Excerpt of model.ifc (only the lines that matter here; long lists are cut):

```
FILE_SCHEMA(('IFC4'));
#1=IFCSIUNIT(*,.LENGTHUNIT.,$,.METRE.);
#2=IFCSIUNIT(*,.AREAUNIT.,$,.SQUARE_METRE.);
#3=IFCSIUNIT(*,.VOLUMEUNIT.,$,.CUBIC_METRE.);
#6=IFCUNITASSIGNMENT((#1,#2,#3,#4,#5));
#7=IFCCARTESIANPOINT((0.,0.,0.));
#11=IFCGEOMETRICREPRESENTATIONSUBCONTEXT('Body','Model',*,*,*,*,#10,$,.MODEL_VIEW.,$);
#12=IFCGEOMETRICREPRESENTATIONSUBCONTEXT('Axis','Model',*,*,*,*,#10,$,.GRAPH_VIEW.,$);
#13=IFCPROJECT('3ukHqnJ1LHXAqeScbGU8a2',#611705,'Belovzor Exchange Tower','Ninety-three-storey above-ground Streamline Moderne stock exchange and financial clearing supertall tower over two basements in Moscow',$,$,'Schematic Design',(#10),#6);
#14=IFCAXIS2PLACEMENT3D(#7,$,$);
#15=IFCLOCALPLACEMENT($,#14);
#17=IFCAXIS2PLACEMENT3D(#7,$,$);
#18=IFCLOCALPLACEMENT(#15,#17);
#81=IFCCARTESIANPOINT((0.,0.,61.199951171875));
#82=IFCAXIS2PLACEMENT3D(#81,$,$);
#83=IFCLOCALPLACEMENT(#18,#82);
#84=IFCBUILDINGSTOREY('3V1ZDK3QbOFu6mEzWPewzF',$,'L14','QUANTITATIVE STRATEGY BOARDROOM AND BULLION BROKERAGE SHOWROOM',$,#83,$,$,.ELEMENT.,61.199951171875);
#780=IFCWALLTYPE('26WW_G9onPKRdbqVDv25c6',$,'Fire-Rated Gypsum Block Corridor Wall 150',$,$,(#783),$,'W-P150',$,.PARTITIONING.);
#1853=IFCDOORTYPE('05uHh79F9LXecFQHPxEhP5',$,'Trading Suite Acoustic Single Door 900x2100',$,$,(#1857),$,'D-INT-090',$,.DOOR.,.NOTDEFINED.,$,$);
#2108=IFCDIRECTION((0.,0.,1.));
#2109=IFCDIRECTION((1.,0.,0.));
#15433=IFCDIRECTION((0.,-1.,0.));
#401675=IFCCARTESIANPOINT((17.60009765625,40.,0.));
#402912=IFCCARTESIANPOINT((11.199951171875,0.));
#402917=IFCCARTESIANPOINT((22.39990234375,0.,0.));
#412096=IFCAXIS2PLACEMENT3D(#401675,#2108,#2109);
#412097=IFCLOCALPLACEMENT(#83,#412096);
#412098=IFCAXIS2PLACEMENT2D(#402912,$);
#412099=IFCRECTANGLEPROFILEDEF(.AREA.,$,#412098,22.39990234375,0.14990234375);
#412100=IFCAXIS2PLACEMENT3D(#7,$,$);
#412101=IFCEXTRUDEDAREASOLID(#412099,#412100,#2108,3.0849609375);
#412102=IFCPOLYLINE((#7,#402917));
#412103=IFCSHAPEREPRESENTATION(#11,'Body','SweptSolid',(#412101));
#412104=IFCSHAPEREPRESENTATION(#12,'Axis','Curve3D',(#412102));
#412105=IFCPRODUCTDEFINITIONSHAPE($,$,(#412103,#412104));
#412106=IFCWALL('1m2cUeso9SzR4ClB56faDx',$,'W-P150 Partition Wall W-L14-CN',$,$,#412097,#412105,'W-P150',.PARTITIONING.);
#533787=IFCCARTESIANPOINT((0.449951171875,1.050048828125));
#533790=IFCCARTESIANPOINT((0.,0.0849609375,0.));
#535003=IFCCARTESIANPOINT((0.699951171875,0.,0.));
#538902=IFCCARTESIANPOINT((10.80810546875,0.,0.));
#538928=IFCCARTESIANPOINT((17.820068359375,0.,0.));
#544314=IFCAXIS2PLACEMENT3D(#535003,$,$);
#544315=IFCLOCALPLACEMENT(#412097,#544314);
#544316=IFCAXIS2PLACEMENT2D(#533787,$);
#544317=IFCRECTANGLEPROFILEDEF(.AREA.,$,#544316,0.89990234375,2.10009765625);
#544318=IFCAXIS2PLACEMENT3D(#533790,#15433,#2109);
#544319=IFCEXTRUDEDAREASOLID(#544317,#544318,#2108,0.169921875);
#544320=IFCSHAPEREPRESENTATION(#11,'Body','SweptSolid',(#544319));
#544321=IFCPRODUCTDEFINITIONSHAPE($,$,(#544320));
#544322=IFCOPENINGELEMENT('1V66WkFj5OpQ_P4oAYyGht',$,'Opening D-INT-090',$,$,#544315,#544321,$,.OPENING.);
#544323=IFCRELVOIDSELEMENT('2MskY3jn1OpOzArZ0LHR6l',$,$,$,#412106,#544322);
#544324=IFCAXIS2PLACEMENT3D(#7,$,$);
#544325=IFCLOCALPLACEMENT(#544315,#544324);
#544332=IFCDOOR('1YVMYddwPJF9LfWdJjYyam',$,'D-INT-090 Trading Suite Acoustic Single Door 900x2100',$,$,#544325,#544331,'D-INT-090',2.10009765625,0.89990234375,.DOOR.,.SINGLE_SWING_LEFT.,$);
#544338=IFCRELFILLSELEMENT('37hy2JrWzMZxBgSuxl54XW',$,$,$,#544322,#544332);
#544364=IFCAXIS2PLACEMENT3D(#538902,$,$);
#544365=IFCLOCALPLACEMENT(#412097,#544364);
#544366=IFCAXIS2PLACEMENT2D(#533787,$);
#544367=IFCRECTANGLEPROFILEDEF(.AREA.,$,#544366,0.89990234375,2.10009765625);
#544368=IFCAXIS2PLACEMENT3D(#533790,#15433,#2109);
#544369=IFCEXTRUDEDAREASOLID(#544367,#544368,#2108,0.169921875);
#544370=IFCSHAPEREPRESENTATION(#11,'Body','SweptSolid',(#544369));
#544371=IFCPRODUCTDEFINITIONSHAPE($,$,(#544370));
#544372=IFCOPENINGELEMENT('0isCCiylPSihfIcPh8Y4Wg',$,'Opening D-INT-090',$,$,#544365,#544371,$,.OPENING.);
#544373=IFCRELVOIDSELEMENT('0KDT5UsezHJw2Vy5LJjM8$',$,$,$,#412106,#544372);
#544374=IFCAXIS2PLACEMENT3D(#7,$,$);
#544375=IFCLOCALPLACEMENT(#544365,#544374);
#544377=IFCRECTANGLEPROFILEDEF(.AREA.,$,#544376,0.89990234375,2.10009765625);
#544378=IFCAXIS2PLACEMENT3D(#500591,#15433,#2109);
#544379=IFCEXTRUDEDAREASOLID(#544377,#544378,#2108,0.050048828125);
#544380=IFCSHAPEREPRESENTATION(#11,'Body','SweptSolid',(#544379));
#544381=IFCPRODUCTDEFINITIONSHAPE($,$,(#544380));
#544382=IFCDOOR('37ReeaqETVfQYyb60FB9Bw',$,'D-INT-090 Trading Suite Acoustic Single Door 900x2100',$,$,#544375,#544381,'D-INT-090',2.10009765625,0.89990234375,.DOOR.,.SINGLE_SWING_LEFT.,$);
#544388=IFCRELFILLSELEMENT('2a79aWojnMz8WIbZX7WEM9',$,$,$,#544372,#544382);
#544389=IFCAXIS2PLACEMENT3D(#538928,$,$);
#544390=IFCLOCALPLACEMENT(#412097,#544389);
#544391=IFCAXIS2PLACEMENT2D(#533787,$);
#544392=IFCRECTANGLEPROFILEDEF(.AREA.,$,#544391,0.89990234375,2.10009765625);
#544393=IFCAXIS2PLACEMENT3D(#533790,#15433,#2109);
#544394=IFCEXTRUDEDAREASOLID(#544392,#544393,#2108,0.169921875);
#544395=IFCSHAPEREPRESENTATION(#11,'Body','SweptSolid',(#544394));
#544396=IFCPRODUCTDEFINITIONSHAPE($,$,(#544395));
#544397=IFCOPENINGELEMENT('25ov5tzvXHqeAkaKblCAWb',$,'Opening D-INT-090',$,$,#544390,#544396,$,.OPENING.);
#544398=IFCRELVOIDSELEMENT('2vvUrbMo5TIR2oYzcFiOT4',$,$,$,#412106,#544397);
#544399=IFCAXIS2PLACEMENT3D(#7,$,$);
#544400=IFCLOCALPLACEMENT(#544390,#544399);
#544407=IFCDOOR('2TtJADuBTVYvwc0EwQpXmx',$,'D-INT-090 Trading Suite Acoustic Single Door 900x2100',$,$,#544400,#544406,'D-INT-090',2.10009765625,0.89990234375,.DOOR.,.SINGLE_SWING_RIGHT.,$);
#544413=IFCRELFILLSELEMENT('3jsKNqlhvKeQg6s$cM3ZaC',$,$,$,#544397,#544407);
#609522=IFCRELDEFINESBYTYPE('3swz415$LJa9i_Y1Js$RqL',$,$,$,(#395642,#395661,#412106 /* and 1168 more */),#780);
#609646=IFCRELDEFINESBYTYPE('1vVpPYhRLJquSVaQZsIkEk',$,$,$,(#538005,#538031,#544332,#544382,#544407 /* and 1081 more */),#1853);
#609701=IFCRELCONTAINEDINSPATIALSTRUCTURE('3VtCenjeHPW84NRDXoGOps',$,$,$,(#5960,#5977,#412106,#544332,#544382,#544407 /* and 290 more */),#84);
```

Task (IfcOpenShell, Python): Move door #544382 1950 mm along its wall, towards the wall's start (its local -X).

```python
import ifcopenshell
import ifcopenshell.api.geometry
import ifcopenshell.util.placement
import ifcopenshell.util.unit

model = ifcopenshell.open("model.ifc")
unit_scale = ifcopenshell.util.unit.calculate_unit_scale(model)

door = model.by_guid("37ReeaqETVfQYyb60FB9Bw")
opening = door.FillsVoids[0].RelatingOpeningElement
wall = opening.VoidsElements[0].RelatingBuildingElement

wall_matrix = ifcopenshell.util.placement.get_local_placement(wall.ObjectPlacement)
shift = wall_matrix[:3, 0] * -1.95 / unit_scale
before = ifcopenshell.util.placement.get_local_placement(door.ObjectPlacement)[:3, 3].copy()

# The door is placed relative to its opening, so it follows when the opening moves.
matrix = ifcopenshell.util.placement.get_local_placement(opening.ObjectPlacement)
matrix[:3, 3] += shift
ifcopenshell.api.geometry.edit_object_placement(
    model, product=opening, matrix=matrix, is_si=False, should_transform_children=True
)

after = ifcopenshell.util.placement.get_local_placement(door.ObjectPlacement)[:3, 3]
print("door moved by", (after - before).round(3) + 0.0)

model.write("model-out.ifc")
```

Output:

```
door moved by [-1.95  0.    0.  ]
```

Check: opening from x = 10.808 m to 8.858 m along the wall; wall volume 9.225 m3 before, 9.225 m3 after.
